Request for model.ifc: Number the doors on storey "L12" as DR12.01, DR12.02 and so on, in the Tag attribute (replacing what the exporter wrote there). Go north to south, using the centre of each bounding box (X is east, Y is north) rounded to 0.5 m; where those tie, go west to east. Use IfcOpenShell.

First a look at what the model holds.

```python
import ifcopenshell
import ifcopenshell.util.element
import ifcopenshell.util.placement

model = ifcopenshell.open("model.ifc")
print(model.schema)
storey = next(s for s in model.by_type("IfcBuildingStorey") if s.Name == "L12")
doors = [e for e in ifcopenshell.util.element.get_decomposition(storey) if e.is_a("IfcDoor")]
for e in sorted(doors, key=lambda e: e.id()):
    origin = ifcopenshell.util.placement.get_local_placement(e.ObjectPlacement)[:3, 3]
    print(e.id(), e.Tag, e.Name, origin.round(2) + 0.0, sep=" | ")
```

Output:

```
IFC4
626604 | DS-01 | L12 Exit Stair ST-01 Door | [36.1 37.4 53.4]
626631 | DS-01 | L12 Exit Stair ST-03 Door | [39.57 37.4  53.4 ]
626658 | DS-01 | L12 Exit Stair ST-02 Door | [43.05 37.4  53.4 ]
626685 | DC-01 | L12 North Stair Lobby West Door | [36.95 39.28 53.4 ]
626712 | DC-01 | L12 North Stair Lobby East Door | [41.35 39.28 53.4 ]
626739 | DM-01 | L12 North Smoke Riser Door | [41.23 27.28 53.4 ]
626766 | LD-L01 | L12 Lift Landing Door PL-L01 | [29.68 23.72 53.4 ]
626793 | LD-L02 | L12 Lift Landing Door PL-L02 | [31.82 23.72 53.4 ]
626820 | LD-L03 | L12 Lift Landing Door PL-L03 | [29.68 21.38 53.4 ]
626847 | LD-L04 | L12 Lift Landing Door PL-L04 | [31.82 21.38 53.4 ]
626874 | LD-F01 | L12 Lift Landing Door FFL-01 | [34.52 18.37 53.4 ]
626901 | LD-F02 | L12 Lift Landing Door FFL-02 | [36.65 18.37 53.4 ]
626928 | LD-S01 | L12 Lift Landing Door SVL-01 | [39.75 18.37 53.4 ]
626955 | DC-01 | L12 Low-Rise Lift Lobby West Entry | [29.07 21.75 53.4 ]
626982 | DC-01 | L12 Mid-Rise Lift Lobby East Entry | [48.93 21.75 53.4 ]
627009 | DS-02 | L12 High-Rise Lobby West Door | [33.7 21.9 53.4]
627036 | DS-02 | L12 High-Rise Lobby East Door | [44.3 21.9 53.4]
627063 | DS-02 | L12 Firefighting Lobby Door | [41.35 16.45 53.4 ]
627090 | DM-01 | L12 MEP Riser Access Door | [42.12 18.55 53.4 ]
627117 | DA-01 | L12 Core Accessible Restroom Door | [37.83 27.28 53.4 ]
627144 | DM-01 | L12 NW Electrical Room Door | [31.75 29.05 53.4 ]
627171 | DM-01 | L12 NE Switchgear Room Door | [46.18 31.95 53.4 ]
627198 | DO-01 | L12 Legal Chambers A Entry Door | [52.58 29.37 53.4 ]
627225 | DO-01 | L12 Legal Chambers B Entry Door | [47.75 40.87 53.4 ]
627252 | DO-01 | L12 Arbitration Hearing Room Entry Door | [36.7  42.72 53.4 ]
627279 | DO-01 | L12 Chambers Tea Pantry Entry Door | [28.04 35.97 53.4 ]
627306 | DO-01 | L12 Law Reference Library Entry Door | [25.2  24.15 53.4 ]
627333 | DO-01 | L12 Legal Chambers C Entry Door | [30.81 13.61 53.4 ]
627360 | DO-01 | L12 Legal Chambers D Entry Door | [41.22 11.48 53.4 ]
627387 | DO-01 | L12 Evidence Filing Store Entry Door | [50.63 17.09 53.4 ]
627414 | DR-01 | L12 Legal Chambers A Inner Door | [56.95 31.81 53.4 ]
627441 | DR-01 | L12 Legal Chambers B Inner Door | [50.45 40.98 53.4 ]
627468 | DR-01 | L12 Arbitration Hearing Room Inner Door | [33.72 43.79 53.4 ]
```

```python
import ifcopenshell
import ifcopenshell.geom
import ifcopenshell.util.element
import ifcopenshell.util.shape

model = ifcopenshell.open("model.ifc")
settings = ifcopenshell.geom.settings()
settings.set("use-world-coords", True)


def centre(element):
    shape = ifcopenshell.geom.create_shape(settings, element)
    return ifcopenshell.util.shape.get_bbox_centroid(shape.geometry)


storey = next(s for s in model.by_type("IfcBuildingStorey") if s.Name == "L12")
doors = [e for e in ifcopenshell.util.element.get_decomposition(storey) if e.is_a("IfcDoor")]

# Insertion points can sit at a corner or the storey origin, so sort by the geometry (in metres).
centres = {e: centre(e) for e in doors}
doors.sort(key=lambda e: (-round(centres[e][1] / 0.5), centres[e][0]))

for i, e in enumerate(doors, start=1):
    number = f"DR12.{i:02d}"
    e.Tag = number
    print(e.id(), number)

model.write("model-out.ifc")
```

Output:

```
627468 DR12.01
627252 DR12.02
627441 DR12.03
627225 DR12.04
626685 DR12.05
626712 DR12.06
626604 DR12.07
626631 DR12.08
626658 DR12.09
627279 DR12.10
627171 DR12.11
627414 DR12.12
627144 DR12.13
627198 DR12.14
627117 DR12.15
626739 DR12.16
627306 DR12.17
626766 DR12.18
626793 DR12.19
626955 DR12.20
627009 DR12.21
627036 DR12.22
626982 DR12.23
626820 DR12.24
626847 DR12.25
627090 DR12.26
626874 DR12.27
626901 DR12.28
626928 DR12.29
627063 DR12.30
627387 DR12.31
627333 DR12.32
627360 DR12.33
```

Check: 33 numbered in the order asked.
